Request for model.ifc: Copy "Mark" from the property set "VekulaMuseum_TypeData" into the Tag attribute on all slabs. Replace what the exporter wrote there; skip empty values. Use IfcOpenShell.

First a look at what the model holds.

```python
import ifcopenshell
import ifcopenshell.util.element

model = ifcopenshell.open("model.ifc")
print(model.schema)
slabs = model.by_type("IfcSlab")
print(len(slabs), "slabs")
for e in slabs[:8]:
    source = ifcopenshell.util.element.get_pset(e, "VekulaMuseum_TypeData", "Mark")
    target = e.Tag
    print(e.id(), repr(source), repr(target), sep=" | ")
```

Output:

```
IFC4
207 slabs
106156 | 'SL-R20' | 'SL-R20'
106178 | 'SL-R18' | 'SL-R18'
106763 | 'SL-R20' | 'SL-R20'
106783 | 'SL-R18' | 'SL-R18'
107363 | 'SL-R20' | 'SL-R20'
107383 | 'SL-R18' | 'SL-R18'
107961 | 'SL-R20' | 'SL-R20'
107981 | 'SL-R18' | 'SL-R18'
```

```python
import ifcopenshell
import ifcopenshell.util.element

model = ifcopenshell.open("model.ifc")

count = 0
for e in model.by_type("IfcSlab"):
    value = ifcopenshell.util.element.get_pset(e, "VekulaMuseum_TypeData", "Mark")
    current = e.Tag
    if not value or not value.strip() or current == value:
        continue
    e.Tag = value
    count += 1

print(count, "slabs updated")

model.write("model_rev.ifc")
```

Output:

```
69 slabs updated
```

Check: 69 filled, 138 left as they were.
